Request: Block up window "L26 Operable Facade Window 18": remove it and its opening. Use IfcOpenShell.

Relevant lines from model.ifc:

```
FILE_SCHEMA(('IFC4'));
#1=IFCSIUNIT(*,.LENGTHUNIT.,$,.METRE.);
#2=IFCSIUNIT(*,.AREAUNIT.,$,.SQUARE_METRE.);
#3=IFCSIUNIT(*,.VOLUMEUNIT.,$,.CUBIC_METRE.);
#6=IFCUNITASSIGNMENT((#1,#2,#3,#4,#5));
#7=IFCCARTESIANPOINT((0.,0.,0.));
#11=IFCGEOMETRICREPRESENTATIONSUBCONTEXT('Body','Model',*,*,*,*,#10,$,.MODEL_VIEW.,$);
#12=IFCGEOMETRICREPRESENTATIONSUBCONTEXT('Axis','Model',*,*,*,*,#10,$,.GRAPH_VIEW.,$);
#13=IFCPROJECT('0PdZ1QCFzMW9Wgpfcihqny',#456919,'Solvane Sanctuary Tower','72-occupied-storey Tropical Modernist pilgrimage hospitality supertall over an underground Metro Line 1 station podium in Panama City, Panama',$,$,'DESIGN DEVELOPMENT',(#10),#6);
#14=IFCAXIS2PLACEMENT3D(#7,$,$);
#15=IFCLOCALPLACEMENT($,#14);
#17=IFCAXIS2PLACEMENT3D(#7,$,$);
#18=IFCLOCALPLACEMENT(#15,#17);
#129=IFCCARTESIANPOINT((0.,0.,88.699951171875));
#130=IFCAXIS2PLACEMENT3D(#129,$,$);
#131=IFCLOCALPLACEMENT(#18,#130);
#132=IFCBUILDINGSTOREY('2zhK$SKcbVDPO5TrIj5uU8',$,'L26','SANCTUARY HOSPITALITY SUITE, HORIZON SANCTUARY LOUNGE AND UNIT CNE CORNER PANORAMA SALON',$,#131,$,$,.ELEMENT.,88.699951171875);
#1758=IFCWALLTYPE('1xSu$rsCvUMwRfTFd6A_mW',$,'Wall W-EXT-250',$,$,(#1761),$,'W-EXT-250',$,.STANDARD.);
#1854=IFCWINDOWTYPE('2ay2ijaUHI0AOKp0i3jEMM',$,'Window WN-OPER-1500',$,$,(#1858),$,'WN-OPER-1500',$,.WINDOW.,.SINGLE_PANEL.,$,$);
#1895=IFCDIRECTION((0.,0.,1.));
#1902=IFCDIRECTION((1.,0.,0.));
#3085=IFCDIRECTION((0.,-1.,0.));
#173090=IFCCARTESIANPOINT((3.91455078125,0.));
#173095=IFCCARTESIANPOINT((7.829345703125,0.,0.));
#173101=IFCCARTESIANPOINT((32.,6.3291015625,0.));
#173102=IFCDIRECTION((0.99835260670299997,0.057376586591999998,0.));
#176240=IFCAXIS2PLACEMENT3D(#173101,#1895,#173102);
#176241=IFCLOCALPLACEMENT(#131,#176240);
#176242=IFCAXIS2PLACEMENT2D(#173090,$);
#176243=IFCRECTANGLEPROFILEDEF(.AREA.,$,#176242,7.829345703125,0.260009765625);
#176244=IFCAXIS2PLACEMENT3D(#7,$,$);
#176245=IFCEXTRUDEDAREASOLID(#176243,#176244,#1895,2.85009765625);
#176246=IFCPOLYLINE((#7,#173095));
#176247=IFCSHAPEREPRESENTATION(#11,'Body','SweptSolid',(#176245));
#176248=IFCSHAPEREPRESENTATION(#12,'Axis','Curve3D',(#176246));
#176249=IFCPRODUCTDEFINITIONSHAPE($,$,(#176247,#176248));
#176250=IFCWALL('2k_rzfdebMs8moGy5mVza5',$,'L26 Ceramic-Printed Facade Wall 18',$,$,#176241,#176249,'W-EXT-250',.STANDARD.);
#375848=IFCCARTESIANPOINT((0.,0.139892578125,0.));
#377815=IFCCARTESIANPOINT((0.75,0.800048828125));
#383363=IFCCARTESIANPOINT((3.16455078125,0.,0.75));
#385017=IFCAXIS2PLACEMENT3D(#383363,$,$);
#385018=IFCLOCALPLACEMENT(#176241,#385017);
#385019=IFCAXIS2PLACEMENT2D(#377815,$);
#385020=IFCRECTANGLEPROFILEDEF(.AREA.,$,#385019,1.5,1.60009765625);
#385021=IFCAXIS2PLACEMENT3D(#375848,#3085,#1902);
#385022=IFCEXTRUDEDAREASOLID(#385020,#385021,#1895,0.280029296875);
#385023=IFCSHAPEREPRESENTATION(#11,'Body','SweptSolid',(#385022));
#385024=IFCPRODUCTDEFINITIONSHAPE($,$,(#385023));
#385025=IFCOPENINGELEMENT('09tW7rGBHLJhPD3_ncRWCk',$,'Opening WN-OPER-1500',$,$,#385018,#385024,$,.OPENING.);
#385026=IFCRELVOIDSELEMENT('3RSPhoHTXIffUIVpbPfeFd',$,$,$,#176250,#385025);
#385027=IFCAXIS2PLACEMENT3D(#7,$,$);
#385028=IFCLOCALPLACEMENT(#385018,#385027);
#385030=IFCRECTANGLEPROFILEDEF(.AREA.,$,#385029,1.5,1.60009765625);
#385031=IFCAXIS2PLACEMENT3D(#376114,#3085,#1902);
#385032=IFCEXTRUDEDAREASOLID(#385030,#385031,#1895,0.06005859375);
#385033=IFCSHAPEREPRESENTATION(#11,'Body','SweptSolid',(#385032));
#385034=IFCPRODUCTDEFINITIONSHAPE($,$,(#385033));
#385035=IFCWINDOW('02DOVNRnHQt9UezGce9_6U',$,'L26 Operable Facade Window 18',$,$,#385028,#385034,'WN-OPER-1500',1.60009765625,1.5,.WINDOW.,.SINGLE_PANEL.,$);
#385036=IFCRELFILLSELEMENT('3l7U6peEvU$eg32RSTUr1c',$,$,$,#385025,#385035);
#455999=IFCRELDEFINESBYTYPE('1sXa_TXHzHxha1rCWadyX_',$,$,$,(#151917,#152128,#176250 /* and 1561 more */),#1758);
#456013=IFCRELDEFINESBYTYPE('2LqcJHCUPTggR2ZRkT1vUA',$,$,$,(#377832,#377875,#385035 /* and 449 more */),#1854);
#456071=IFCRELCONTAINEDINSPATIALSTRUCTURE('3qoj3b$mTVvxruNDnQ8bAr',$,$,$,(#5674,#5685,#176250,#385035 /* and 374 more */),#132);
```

```python
import ifcopenshell
import ifcopenshell.api.feature
import ifcopenshell.api.root
import ifcopenshell.geom
import ifcopenshell.util.shape

model = ifcopenshell.open("model.ifc")
settings = ifcopenshell.geom.settings()


def volume(element):
    """Net volume in cubic metres, openings subtracted."""
    shape = ifcopenshell.geom.create_shape(settings, element)
    return ifcopenshell.util.shape.get_volume(shape.geometry)


window = model.by_guid("02DOVNRnHQt9UezGce9_6U")
opening = window.FillsVoids[0].RelatingOpeningElement
wall = opening.VoidsElements[0].RelatingBuildingElement
before = volume(wall)

ifcopenshell.api.root.remove_product(model, product=window)
ifcopenshell.api.feature.remove_feature(model, feature=opening)

after = volume(wall)

print(f"wall volume {before:.3f} -> {after:.3f} m3")

model.write("model_rev.ifc")
```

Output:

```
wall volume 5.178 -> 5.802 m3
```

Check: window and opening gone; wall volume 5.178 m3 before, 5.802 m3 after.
